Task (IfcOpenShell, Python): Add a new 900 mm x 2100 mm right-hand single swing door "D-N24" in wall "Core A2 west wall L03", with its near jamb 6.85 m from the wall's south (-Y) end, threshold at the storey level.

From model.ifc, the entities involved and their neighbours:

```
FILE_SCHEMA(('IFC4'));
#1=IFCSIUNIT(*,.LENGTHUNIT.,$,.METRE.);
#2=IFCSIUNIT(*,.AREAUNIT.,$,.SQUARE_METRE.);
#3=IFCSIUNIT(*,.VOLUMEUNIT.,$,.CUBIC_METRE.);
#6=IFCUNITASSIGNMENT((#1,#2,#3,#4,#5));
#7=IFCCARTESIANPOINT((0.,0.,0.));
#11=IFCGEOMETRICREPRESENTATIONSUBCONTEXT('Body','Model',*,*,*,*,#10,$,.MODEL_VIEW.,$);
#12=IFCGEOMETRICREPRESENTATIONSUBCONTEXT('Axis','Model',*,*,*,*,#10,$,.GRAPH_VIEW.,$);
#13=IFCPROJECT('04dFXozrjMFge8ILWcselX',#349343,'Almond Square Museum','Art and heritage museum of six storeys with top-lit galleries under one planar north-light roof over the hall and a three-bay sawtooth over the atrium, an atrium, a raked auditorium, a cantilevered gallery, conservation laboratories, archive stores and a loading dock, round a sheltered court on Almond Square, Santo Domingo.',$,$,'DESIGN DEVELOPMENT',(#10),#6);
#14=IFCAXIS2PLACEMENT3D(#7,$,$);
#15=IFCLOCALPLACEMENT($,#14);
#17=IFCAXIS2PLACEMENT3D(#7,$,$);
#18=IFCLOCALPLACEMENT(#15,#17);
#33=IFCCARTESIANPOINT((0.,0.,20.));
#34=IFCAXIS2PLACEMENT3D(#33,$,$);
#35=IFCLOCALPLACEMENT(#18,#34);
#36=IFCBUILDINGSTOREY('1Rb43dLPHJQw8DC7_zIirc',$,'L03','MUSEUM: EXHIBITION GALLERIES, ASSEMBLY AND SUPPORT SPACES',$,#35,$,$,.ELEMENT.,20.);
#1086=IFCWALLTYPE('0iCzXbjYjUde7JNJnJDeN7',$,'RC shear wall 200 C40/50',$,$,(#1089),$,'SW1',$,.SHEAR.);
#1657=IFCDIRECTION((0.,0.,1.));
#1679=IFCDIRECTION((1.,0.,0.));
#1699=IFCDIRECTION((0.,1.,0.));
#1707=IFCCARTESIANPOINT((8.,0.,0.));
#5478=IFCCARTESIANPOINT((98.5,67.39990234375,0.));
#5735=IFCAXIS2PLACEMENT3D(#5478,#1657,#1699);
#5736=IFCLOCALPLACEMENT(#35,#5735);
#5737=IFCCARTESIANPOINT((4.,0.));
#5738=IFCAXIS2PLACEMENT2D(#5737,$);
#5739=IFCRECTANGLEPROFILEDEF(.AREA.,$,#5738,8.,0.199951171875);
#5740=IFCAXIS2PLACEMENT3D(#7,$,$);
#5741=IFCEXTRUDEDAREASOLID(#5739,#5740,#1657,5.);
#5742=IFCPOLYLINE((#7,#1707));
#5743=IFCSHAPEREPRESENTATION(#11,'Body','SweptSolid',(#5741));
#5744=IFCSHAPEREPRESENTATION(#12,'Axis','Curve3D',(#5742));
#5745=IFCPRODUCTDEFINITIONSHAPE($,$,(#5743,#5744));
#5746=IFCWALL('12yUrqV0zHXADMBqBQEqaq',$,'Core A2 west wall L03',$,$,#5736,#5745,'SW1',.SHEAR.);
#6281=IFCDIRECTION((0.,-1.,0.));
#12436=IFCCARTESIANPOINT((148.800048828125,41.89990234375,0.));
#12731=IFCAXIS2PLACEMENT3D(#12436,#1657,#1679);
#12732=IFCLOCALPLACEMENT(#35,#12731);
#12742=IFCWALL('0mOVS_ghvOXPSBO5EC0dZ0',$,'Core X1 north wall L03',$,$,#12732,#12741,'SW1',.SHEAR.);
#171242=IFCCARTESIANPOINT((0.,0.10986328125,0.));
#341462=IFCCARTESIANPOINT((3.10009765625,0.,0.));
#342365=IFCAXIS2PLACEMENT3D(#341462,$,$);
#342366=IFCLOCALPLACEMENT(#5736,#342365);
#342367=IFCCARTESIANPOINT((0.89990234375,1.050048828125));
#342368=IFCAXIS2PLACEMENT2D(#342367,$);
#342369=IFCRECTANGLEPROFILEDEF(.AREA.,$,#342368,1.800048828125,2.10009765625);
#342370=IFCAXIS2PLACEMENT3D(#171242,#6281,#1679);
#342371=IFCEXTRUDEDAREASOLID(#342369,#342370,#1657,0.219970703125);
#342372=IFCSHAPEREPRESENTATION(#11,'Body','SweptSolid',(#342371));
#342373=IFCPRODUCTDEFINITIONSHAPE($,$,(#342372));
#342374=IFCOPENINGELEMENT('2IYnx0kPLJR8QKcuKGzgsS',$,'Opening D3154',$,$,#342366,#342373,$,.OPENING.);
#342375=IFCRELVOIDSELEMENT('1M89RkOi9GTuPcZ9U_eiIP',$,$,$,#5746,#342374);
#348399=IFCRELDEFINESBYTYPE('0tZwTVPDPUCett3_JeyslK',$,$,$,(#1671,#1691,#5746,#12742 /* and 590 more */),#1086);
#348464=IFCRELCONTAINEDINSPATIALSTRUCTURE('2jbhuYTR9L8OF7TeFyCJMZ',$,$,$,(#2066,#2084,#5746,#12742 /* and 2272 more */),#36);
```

```python
import numpy as np
import ifcopenshell
import ifcopenshell.api.feature
import ifcopenshell.api.geometry
import ifcopenshell.api.root
import ifcopenshell.api.spatial
import ifcopenshell.geom
import ifcopenshell.util.element
import ifcopenshell.util.placement
import ifcopenshell.util.representation
import ifcopenshell.util.shape
import ifcopenshell.util.unit

model = ifcopenshell.open("model.ifc")
unit_scale = ifcopenshell.util.unit.calculate_unit_scale(model)
settings = ifcopenshell.geom.settings()


def volume(element):
    """Net volume in cubic metres, openings subtracted."""
    shape = ifcopenshell.geom.create_shape(settings, element)
    return ifcopenshell.util.shape.get_volume(shape.geometry)


wall = model.by_id(5746)
storey = ifcopenshell.util.element.get_container(wall, ifc_class="IfcBuildingStorey")
context = ifcopenshell.util.representation.get_context(model, "Model", "Body", "MODEL_VIEW")
before = volume(wall)

width, height, from_end, sill = 0.9, 2.1, 6.85, 0.0  # metres

# The wall runs along its own X axis, and the end named is its -X end.
wall_shape = ifcopenshell.geom.create_shape(settings, wall)
x, y, z = ifcopenshell.util.shape.get_vertices(wall_shape.geometry).T
start = x.min() + from_end
face, thickness = float(y.min()), float(y.max() - y.min())
wall_matrix = ifcopenshell.util.placement.get_local_placement(wall.ObjectPlacement)
level = ifcopenshell.util.placement.get_local_placement(storey.ObjectPlacement)[2, 3]


def in_wall(x, y):
    """Placement at x, y metres in the wall's axes, at sill height."""
    matrix = wall_matrix.copy()
    matrix[:, 3] = wall_matrix @ np.array([x / unit_scale, y / unit_scale, 0.0, 1.0])
    matrix[2, 3] = level + sill / unit_scale
    return matrix


# Opening: a box that overshoots both wall faces by 50 mm.
opening = ifcopenshell.api.root.create_entity(model, ifc_class="IfcOpeningElement", predefined_type="OPENING")
box = ifcopenshell.api.geometry.add_wall_representation(
    model, context=context, length=width, height=height, thickness=thickness + 0.1
)
ifcopenshell.api.geometry.assign_representation(model, product=opening, representation=box)
ifcopenshell.api.geometry.edit_object_placement(model, product=opening, matrix=in_wall(start, face - 0.05), is_si=False)
ifcopenshell.api.feature.add_feature(model, feature=opening, element=wall)

door = ifcopenshell.api.root.create_entity(model, ifc_class="IfcDoor", name="D-N24", predefined_type="DOOR")
door.OverallWidth, door.OverallHeight = width / unit_scale, height / unit_scale
door.OperationType = "SINGLE_SWING_RIGHT"
body = ifcopenshell.api.geometry.add_door_representation(
    model,
    context=context,
    overall_width=door.OverallWidth,
    overall_height=door.OverallHeight,
    operation_type="SINGLE_SWING_RIGHT",
    lining_properties={"LiningDepth": thickness / unit_scale, "ThresholdDepth": thickness / unit_scale},
)
ifcopenshell.api.geometry.assign_representation(model, product=door, representation=body)
ifcopenshell.api.spatial.assign_container(model, products=[door], relating_structure=storey)
ifcopenshell.api.feature.add_filling(model, opening=opening, element=door)

# The lining spans the wall, so the door starts at the wall face.
ifcopenshell.api.geometry.edit_object_placement(model, product=door, matrix=in_wall(start, face), is_si=False)

after = volume(wall)

print(f"wall volume {before:.3f} -> {after:.3f} m3")

model.write("model-out.ifc")
```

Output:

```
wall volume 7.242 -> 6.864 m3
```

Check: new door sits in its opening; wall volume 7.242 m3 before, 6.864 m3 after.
